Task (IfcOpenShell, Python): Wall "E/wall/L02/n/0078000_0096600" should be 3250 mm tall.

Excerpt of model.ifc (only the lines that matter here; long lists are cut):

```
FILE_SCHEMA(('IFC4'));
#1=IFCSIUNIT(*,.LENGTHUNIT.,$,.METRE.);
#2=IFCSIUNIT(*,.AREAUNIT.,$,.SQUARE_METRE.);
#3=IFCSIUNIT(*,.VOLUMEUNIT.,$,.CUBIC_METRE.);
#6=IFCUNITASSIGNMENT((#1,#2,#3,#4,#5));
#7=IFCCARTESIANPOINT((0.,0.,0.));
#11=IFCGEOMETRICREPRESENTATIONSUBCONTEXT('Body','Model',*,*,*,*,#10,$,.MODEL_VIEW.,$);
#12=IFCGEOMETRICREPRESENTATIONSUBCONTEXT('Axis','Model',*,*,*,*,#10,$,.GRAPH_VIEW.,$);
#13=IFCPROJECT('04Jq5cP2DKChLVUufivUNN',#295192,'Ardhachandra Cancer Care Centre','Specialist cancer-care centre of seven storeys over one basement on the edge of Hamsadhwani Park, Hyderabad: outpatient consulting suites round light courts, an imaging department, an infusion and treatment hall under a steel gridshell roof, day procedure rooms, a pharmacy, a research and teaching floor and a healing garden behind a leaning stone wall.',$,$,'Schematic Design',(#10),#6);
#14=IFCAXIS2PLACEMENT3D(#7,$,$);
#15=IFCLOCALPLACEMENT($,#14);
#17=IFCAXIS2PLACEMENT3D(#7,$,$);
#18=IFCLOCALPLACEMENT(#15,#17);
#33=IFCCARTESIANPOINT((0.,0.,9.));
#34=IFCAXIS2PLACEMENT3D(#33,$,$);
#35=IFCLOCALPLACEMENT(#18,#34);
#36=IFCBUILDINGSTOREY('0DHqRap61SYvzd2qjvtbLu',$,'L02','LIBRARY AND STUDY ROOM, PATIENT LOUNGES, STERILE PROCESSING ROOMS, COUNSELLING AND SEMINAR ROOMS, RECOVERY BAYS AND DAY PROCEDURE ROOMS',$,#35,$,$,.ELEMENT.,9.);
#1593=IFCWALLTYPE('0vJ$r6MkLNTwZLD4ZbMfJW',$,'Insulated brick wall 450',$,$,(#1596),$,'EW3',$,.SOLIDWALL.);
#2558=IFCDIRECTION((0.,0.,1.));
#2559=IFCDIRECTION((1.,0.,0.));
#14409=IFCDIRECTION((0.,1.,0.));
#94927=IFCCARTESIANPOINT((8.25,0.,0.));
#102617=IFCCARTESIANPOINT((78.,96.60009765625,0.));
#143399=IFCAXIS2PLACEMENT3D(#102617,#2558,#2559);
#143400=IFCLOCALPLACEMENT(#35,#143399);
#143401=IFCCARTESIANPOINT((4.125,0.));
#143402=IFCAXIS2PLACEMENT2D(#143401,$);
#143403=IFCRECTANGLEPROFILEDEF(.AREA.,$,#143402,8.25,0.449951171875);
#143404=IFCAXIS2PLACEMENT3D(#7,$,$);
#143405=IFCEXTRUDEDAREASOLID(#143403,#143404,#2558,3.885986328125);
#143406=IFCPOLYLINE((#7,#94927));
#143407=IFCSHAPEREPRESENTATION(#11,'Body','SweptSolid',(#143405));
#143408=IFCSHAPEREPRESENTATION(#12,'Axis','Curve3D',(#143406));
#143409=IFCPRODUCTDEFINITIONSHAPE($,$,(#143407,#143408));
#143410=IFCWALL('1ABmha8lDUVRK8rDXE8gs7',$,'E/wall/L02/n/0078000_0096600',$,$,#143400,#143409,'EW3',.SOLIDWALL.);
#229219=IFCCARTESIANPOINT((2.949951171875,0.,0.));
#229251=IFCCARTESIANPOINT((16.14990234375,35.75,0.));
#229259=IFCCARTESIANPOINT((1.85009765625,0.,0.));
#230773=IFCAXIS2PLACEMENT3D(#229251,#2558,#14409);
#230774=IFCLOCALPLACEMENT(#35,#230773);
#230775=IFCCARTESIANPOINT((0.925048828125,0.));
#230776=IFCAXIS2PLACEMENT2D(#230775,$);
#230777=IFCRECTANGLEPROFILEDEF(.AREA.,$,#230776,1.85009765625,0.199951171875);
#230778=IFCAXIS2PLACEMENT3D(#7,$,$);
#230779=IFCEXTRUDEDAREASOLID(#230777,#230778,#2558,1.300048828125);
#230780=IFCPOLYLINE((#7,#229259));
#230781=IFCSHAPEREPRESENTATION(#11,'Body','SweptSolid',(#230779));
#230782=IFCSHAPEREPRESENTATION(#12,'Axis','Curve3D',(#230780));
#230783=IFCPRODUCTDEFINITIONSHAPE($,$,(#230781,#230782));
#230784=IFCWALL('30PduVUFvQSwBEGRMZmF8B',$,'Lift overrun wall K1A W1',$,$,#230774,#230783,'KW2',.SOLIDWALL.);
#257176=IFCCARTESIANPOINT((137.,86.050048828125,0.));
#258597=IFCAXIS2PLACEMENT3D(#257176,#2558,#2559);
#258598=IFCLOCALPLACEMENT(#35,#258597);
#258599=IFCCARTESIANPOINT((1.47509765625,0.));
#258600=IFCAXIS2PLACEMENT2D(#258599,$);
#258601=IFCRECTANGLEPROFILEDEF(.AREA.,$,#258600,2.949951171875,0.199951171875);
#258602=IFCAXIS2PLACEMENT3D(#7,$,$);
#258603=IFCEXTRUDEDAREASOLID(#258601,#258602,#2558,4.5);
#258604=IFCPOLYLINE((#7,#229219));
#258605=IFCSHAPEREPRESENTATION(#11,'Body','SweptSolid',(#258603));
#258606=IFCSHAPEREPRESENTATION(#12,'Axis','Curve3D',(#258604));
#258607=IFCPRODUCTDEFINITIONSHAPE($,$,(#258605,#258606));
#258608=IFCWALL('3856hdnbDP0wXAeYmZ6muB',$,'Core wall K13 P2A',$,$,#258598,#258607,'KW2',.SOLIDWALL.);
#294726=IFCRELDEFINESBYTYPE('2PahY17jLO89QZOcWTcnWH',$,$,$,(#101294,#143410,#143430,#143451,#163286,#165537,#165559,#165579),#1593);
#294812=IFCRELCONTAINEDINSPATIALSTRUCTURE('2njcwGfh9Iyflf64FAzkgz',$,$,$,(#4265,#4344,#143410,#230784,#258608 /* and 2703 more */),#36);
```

```python
import ifcopenshell
import ifcopenshell.geom
import ifcopenshell.util.representation
import ifcopenshell.util.shape
import ifcopenshell.util.unit

model = ifcopenshell.open("model.ifc")
unit_scale = ifcopenshell.util.unit.calculate_unit_scale(model)
settings = ifcopenshell.geom.settings()


def volume(element):
    """Net volume in cubic metres, openings subtracted."""
    shape = ifcopenshell.geom.create_shape(settings, element)
    return ifcopenshell.util.shape.get_volume(shape.geometry)


wall = model.by_guid("1ABmha8lDUVRK8rDXE8gs7")
before = volume(wall)

body = ifcopenshell.util.representation.get_representation(wall, "Model", "Body")
solid = body.Items[0]
old_height = solid.Depth
solid.Depth = 3.25 / unit_scale
after = volume(wall)

print(f"height {old_height:g} -> {solid.Depth:g}, volume {before:.3f} -> {after:.3f} m3")

model.write("model_updated.ifc")
```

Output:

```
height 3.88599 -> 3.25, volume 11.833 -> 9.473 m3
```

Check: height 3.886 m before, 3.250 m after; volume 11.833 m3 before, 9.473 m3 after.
